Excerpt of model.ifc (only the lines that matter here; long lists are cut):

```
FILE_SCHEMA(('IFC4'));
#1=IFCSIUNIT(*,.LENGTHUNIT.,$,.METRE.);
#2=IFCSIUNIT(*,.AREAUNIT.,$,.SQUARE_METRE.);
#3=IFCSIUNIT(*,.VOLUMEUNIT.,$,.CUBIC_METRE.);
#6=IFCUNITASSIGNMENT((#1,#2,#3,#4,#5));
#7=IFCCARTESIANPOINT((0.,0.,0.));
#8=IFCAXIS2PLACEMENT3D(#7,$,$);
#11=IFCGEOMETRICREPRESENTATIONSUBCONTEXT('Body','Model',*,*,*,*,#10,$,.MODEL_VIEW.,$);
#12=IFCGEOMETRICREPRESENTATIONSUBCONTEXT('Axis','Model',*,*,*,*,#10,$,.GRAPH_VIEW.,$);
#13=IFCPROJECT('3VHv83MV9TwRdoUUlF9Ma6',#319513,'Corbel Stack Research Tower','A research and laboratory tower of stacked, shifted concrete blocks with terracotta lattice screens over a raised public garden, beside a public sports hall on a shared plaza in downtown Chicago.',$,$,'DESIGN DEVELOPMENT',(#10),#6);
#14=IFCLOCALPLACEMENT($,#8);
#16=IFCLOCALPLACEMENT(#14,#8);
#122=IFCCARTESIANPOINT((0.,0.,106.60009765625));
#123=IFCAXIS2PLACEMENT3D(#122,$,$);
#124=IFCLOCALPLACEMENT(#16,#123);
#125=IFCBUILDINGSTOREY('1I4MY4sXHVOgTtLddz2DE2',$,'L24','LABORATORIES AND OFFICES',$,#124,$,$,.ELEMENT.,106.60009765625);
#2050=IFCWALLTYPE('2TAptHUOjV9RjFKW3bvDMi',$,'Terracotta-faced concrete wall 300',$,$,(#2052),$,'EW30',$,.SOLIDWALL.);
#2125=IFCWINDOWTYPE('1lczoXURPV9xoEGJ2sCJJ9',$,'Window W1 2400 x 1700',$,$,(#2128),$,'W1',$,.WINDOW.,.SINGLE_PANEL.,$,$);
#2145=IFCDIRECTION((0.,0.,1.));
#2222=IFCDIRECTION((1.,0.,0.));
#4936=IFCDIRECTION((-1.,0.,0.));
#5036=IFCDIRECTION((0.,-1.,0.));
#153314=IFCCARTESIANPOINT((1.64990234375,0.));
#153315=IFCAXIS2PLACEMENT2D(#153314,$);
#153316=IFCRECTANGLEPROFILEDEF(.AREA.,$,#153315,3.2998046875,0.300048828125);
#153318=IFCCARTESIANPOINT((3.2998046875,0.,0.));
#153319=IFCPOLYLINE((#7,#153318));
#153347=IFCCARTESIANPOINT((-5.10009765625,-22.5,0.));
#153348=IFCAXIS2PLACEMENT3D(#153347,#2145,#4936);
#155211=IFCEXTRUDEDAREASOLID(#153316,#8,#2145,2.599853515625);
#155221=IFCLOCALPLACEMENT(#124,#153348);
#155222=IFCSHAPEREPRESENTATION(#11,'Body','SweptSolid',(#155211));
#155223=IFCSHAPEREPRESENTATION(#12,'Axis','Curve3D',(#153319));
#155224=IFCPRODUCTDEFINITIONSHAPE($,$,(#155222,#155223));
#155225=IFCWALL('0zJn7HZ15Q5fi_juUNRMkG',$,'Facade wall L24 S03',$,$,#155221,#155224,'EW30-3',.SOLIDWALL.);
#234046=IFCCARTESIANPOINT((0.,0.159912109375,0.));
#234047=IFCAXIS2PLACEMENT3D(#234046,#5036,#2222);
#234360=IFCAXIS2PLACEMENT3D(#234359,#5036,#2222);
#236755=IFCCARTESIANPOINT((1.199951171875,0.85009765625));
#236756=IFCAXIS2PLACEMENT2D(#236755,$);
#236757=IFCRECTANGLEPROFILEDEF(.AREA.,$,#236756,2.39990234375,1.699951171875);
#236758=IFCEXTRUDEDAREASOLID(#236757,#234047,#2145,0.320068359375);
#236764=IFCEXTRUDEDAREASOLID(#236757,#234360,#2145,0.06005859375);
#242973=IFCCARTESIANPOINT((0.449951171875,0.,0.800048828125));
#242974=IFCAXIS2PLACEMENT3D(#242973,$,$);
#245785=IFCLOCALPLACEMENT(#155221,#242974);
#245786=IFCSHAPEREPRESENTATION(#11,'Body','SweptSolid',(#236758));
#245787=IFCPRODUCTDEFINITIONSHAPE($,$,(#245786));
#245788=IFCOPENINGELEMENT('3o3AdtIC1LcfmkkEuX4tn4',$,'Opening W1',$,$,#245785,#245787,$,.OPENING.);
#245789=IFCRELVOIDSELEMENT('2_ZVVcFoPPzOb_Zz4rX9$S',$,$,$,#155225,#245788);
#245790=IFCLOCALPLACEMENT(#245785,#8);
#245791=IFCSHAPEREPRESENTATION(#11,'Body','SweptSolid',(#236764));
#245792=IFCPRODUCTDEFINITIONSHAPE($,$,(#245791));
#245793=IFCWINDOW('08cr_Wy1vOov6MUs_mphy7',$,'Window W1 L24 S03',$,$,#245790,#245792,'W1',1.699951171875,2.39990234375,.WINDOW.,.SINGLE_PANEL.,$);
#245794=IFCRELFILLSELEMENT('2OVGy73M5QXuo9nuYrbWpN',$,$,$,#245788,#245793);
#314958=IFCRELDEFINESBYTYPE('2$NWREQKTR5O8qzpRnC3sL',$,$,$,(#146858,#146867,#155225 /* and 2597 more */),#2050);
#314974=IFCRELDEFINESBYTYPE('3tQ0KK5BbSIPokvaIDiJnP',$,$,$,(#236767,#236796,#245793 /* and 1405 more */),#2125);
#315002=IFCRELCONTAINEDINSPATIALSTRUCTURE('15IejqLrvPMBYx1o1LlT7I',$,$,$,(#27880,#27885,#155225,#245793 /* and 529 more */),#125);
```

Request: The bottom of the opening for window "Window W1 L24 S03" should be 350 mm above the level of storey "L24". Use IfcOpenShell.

```python
import numpy as np
import ifcopenshell
import ifcopenshell.api.geometry
import ifcopenshell.geom
import ifcopenshell.util.element
import ifcopenshell.util.placement
import ifcopenshell.util.shape
import ifcopenshell.util.unit

model = ifcopenshell.open("model.ifc")
unit_scale = ifcopenshell.util.unit.calculate_unit_scale(model)

window = model.by_id(245793)
opening = window.FillsVoids[0].RelatingOpeningElement
storey = ifcopenshell.util.element.get_container(window, ifc_class="IfcBuildingStorey")
level = ifcopenshell.util.placement.get_local_placement(storey.ObjectPlacement)[2, 3]

# The opening's origin need not be at the sill, so measure its lowest point.
shape = ifcopenshell.geom.create_shape(ifcopenshell.geom.settings(), opening)
bottom = ifcopenshell.util.shape.get_shape_bottom_elevation(shape, shape.geometry) / unit_scale
dz = level + 0.35 / unit_scale - bottom

shift = np.array([0.0, 0.0, dz])
# The window is placed relative to its opening, so it follows when the opening moves.
matrix = ifcopenshell.util.placement.get_local_placement(opening.ObjectPlacement)
matrix[:3, 3] += shift
ifcopenshell.api.geometry.edit_object_placement(
    model, product=opening, matrix=matrix, is_si=False, should_transform_children=True
)

print(f"moved by {dz * unit_scale:+.3f} m")

model.write("model-out.ifc")
```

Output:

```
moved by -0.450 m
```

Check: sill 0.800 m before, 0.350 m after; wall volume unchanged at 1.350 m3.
